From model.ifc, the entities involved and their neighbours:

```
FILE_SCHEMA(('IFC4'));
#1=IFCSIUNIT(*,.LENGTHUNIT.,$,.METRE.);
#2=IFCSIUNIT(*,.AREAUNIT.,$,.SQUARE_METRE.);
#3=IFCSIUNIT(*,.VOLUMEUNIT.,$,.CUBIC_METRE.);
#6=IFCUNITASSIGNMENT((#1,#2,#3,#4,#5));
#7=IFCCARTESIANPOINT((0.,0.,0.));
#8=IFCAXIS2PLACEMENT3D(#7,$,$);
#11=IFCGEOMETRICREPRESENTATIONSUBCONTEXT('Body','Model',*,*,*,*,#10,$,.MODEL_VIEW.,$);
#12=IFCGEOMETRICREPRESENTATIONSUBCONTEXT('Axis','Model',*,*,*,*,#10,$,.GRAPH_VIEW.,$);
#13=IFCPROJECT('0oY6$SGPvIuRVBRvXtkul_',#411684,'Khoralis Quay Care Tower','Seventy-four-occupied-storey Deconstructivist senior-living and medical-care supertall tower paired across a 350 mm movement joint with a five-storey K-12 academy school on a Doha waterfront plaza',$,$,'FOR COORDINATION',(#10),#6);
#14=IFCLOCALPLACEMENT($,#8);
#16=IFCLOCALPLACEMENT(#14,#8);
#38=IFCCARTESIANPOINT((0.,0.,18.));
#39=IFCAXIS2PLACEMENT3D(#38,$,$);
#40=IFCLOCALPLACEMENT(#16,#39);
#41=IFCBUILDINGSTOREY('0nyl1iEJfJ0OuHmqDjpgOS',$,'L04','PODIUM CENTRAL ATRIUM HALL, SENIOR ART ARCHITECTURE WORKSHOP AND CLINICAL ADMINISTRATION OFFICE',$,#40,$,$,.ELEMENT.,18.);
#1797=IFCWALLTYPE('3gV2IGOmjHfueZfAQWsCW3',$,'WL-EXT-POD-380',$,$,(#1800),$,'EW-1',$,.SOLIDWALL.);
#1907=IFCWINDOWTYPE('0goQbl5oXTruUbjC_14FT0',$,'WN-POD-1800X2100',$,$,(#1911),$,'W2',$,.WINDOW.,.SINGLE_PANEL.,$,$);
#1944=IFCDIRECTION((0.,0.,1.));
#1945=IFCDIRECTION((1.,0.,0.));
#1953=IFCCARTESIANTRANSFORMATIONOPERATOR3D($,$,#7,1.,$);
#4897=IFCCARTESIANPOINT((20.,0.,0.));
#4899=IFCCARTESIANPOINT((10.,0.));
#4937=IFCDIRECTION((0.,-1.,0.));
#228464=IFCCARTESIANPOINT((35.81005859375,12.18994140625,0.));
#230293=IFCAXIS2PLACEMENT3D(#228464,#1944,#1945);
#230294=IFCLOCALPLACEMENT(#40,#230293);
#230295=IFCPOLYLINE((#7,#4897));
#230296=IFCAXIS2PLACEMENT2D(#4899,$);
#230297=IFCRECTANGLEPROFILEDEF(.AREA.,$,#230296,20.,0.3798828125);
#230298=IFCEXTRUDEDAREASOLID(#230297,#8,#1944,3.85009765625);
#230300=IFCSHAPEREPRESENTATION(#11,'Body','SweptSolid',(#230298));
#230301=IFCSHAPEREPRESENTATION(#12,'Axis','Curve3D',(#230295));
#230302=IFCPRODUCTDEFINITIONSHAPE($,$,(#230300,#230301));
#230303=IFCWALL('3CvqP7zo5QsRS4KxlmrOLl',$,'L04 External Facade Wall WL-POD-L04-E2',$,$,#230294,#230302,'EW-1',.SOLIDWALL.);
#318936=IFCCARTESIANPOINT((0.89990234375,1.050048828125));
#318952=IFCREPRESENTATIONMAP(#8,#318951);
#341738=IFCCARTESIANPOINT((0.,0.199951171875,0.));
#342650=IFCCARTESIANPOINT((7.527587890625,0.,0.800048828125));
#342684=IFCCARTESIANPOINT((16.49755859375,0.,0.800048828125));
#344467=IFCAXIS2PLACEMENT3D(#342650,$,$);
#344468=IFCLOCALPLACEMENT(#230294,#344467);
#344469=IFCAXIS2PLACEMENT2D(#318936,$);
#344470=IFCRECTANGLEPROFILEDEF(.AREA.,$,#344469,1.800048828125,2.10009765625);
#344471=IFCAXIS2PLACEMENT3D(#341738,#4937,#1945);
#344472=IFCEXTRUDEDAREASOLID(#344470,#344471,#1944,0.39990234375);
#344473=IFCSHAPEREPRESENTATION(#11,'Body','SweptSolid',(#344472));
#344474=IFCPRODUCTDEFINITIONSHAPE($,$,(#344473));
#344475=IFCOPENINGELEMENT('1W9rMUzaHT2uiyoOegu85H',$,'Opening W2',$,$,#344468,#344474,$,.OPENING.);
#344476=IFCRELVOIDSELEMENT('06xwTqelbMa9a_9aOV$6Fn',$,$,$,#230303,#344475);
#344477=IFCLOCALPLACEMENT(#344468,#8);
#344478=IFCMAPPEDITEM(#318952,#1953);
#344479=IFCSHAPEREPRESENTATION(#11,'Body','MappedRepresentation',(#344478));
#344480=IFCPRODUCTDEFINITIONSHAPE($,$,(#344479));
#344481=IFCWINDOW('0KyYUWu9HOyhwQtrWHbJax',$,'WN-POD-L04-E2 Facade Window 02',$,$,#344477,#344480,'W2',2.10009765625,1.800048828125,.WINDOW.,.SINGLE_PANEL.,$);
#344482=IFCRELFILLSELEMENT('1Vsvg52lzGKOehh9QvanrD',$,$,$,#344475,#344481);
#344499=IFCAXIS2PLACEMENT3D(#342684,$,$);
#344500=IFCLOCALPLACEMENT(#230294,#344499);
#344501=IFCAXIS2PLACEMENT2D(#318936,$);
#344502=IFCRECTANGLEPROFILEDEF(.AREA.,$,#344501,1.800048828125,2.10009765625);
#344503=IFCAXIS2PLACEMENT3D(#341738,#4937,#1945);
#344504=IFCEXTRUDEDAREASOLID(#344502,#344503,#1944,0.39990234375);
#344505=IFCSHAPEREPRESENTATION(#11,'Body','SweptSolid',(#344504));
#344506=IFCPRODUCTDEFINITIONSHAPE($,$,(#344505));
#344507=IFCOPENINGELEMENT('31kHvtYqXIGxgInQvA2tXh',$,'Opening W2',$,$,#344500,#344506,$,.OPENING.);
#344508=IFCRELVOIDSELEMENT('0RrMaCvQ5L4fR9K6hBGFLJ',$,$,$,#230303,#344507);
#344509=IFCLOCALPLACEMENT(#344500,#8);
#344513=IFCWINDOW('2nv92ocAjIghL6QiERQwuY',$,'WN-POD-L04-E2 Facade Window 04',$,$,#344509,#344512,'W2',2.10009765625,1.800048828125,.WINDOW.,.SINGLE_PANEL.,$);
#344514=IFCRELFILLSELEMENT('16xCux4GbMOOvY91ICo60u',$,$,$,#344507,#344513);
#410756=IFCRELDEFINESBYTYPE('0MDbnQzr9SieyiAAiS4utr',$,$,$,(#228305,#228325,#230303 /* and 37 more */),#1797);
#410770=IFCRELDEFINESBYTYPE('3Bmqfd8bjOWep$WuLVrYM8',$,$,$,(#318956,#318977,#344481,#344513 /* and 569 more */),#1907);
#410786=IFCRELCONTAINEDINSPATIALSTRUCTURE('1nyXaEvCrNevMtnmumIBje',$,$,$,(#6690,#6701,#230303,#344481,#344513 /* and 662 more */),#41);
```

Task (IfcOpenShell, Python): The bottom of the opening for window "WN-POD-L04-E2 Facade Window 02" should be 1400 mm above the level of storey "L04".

```python
import numpy as np
import ifcopenshell
import ifcopenshell.api.geometry
import ifcopenshell.geom
import ifcopenshell.util.element
import ifcopenshell.util.placement
import ifcopenshell.util.shape
import ifcopenshell.util.unit

model = ifcopenshell.open("model.ifc")
unit_scale = ifcopenshell.util.unit.calculate_unit_scale(model)

window = model.by_guid("0KyYUWu9HOyhwQtrWHbJax")
opening = window.FillsVoids[0].RelatingOpeningElement
storey = ifcopenshell.util.element.get_container(window, ifc_class="IfcBuildingStorey")
level = ifcopenshell.util.placement.get_local_placement(storey.ObjectPlacement)[2, 3]

# The opening's origin need not be at the sill, so measure its lowest point.
shape = ifcopenshell.geom.create_shape(ifcopenshell.geom.settings(), opening)
bottom = ifcopenshell.util.shape.get_shape_bottom_elevation(shape, shape.geometry) / unit_scale
dz = level + 1.4 / unit_scale - bottom

shift = np.array([0.0, 0.0, dz])
# The window is placed relative to its opening, so it follows when the opening moves.
matrix = ifcopenshell.util.placement.get_local_placement(opening.ObjectPlacement)
matrix[:3, 3] += shift
ifcopenshell.api.geometry.edit_object_placement(
    model, product=opening, matrix=matrix, is_si=False, should_transform_children=True
)

print(f"moved by {dz * unit_scale:+.3f} m")

model.write("model_v2.ifc")
```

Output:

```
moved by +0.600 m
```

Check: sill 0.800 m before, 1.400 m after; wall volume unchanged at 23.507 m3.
